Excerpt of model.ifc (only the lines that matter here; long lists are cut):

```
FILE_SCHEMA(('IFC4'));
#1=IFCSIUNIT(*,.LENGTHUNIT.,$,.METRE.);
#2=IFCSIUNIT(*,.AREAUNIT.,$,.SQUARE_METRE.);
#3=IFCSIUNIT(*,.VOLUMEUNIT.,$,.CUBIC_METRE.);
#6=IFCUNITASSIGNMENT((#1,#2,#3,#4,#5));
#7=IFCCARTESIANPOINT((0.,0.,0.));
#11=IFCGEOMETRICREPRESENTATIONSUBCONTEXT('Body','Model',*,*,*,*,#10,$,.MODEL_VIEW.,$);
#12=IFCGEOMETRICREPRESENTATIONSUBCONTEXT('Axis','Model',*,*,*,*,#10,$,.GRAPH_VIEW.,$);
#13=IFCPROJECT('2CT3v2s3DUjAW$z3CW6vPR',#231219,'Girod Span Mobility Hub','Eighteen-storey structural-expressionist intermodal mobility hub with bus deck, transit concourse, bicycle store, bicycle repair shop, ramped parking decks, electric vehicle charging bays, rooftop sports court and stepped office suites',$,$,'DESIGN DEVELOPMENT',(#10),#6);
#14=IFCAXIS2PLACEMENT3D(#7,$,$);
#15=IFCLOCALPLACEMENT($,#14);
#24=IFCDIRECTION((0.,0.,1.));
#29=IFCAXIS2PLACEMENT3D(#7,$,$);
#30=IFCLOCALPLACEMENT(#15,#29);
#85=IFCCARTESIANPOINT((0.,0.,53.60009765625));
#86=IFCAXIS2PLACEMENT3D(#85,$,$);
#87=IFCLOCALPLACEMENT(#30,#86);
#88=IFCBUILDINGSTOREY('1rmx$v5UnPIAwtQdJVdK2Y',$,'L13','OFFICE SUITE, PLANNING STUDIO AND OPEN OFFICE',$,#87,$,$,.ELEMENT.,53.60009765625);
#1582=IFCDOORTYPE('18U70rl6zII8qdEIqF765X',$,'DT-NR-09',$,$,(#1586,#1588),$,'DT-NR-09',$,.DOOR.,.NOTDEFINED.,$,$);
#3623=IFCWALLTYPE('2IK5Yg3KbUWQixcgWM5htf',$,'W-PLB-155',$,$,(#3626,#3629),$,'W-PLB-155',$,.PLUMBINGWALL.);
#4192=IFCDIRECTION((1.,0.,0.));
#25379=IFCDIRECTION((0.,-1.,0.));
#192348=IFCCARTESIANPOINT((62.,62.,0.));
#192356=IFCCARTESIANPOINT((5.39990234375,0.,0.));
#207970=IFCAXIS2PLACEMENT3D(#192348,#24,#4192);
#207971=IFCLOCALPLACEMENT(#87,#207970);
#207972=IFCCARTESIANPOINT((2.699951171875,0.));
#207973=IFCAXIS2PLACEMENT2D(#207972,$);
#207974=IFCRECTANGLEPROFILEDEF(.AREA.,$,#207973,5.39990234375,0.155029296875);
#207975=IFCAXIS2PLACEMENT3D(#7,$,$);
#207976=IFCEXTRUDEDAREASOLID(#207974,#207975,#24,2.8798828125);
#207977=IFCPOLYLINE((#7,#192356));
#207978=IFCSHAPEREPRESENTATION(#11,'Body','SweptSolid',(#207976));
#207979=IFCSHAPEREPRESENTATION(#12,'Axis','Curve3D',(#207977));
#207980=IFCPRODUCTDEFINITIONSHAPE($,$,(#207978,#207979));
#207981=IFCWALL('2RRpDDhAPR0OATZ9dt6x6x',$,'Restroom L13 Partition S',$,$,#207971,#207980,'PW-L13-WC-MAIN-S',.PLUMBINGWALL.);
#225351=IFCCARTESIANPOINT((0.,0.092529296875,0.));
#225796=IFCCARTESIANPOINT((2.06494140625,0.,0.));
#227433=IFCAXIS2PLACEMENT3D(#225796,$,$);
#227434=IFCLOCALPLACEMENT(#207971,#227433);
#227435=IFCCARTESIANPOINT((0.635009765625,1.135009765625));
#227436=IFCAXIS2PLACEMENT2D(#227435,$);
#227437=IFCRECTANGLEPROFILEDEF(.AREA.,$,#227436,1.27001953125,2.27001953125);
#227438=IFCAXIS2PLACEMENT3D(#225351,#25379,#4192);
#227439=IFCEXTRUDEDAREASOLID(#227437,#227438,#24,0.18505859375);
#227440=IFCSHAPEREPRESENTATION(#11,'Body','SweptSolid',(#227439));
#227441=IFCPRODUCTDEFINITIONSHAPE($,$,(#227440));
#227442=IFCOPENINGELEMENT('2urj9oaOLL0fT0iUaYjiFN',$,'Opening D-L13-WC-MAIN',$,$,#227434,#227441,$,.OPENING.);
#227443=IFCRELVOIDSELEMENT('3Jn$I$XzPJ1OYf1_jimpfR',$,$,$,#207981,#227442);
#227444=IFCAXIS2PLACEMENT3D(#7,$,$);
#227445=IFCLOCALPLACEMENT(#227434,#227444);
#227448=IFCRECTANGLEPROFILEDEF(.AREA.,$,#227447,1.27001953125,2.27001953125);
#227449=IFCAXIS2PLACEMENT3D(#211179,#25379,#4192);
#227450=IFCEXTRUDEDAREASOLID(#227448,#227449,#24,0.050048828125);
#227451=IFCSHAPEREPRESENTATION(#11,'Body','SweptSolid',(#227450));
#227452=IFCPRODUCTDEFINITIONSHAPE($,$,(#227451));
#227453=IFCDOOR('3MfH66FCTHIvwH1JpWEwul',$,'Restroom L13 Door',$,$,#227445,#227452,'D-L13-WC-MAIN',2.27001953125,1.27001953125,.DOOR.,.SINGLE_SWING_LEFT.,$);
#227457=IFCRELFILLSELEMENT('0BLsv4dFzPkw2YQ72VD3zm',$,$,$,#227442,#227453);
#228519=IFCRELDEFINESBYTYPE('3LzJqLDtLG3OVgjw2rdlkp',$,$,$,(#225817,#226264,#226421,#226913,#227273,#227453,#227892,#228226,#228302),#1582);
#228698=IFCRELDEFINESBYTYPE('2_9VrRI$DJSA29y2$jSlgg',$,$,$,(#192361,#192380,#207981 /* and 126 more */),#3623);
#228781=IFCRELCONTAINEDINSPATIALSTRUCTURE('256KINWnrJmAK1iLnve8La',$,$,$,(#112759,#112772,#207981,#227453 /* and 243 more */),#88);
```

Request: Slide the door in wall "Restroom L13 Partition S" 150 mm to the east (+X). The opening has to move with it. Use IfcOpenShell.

```python
import ifcopenshell
import ifcopenshell.api.geometry
import ifcopenshell.util.placement

model = ifcopenshell.open("model.ifc")

door = model.by_guid("3MfH66FCTHIvwH1JpWEwul")
opening = door.FillsVoids[0].RelatingOpeningElement
wall = opening.VoidsElements[0].RelatingBuildingElement

wall_matrix = ifcopenshell.util.placement.get_local_placement(wall.ObjectPlacement)
shift = wall_matrix[:3, 0] * 0.15
before = ifcopenshell.util.placement.get_local_placement(door.ObjectPlacement)[:3, 3].copy()

# The door is placed relative to its opening, so it follows when the opening moves.
matrix = ifcopenshell.util.placement.get_local_placement(opening.ObjectPlacement)
matrix[:3, 3] += shift
ifcopenshell.api.geometry.edit_object_placement(
    model, product=opening, matrix=matrix, is_si=False, should_transform_children=True
)

after = ifcopenshell.util.placement.get_local_placement(door.ObjectPlacement)[:3, 3]
print("door moved by", (after - before).round(3) + 0.0)

model.write("model_updated.ifc")
```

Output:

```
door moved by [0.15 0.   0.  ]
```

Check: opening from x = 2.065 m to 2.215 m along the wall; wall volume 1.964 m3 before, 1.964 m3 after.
